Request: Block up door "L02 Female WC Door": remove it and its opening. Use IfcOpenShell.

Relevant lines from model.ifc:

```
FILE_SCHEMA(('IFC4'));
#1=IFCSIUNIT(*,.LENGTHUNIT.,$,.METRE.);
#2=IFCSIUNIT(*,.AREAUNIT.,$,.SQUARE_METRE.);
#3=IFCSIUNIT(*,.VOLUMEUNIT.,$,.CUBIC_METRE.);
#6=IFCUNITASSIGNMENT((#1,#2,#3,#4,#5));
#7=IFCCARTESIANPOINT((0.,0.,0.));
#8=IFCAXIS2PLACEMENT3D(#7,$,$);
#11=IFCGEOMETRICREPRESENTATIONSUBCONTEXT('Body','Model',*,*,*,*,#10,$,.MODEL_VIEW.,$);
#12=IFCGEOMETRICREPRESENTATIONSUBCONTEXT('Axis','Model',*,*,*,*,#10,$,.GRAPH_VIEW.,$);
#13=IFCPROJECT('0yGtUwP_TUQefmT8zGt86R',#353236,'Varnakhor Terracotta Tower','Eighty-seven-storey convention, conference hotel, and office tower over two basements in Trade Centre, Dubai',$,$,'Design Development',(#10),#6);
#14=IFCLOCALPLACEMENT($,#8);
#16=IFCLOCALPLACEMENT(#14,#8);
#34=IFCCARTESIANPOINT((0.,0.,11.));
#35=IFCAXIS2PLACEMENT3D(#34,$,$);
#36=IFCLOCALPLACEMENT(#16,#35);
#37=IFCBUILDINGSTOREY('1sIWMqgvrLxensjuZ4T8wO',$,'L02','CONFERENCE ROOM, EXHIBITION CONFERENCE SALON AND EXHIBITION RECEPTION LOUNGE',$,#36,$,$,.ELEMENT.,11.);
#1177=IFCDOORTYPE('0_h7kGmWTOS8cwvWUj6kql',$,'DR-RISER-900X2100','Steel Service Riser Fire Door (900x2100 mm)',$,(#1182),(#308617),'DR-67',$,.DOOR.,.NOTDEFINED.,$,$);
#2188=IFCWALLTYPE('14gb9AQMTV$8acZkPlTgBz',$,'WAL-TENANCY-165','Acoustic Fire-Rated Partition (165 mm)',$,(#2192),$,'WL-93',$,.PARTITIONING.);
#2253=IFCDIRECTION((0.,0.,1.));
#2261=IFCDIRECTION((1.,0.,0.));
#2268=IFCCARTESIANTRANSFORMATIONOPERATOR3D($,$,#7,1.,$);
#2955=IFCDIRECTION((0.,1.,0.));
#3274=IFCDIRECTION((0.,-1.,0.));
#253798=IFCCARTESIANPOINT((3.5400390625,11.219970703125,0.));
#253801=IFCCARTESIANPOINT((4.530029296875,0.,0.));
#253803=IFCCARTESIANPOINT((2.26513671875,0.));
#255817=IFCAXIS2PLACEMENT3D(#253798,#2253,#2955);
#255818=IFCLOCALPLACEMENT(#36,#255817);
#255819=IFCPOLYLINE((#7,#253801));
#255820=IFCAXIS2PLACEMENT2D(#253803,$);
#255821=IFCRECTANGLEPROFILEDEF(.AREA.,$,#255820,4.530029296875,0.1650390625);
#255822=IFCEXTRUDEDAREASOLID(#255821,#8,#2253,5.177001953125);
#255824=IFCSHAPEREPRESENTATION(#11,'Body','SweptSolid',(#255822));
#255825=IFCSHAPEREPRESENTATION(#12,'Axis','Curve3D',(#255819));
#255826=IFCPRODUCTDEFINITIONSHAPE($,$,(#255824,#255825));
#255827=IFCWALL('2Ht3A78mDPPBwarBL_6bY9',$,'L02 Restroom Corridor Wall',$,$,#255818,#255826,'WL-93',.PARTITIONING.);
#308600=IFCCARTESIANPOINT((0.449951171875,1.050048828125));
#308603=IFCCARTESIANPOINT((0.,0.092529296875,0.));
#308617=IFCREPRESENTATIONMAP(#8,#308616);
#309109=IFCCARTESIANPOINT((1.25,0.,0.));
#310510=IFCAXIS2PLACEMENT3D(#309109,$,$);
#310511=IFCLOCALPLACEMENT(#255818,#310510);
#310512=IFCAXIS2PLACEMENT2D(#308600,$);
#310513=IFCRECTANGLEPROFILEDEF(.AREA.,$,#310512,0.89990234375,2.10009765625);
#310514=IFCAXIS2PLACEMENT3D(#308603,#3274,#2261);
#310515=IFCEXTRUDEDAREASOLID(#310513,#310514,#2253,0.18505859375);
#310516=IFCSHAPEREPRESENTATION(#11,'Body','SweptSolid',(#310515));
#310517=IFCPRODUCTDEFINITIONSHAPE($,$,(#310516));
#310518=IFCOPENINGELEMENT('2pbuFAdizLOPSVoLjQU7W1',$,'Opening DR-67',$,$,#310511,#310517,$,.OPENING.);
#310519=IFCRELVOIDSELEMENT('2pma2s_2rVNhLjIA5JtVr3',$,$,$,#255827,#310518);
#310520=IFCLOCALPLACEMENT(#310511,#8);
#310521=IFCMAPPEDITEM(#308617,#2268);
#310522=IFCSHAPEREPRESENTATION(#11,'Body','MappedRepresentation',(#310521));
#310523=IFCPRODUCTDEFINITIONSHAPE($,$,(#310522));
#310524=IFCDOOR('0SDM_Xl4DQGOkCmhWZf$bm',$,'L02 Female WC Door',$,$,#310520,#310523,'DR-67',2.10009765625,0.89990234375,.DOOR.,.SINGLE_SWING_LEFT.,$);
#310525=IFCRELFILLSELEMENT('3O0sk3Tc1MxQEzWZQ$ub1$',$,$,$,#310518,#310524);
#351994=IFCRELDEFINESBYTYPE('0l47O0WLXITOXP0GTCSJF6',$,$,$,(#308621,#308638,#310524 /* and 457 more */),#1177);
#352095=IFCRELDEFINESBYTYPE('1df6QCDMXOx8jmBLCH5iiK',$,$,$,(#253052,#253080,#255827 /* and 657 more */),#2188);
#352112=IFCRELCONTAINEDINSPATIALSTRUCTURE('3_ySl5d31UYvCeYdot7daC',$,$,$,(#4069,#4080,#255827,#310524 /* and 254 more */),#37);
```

```python
import ifcopenshell
import ifcopenshell.api.feature
import ifcopenshell.api.root
import ifcopenshell.geom
import ifcopenshell.util.shape

model = ifcopenshell.open("model.ifc")
settings = ifcopenshell.geom.settings()


def volume(element):
    """Net volume in cubic metres, openings subtracted."""
    shape = ifcopenshell.geom.create_shape(settings, element)
    return ifcopenshell.util.shape.get_volume(shape.geometry)


door = model.by_guid("0SDM_Xl4DQGOkCmhWZf$bm")
opening = door.FillsVoids[0].RelatingOpeningElement
wall = opening.VoidsElements[0].RelatingBuildingElement
before = volume(wall)

ifcopenshell.api.root.remove_product(model, product=door)
ifcopenshell.api.feature.remove_feature(model, feature=opening)

after = volume(wall)

print(f"wall volume {before:.3f} -> {after:.3f} m3")

model.write("model_edited.ifc")
```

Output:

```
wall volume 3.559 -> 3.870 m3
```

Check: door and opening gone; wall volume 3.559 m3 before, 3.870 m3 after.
